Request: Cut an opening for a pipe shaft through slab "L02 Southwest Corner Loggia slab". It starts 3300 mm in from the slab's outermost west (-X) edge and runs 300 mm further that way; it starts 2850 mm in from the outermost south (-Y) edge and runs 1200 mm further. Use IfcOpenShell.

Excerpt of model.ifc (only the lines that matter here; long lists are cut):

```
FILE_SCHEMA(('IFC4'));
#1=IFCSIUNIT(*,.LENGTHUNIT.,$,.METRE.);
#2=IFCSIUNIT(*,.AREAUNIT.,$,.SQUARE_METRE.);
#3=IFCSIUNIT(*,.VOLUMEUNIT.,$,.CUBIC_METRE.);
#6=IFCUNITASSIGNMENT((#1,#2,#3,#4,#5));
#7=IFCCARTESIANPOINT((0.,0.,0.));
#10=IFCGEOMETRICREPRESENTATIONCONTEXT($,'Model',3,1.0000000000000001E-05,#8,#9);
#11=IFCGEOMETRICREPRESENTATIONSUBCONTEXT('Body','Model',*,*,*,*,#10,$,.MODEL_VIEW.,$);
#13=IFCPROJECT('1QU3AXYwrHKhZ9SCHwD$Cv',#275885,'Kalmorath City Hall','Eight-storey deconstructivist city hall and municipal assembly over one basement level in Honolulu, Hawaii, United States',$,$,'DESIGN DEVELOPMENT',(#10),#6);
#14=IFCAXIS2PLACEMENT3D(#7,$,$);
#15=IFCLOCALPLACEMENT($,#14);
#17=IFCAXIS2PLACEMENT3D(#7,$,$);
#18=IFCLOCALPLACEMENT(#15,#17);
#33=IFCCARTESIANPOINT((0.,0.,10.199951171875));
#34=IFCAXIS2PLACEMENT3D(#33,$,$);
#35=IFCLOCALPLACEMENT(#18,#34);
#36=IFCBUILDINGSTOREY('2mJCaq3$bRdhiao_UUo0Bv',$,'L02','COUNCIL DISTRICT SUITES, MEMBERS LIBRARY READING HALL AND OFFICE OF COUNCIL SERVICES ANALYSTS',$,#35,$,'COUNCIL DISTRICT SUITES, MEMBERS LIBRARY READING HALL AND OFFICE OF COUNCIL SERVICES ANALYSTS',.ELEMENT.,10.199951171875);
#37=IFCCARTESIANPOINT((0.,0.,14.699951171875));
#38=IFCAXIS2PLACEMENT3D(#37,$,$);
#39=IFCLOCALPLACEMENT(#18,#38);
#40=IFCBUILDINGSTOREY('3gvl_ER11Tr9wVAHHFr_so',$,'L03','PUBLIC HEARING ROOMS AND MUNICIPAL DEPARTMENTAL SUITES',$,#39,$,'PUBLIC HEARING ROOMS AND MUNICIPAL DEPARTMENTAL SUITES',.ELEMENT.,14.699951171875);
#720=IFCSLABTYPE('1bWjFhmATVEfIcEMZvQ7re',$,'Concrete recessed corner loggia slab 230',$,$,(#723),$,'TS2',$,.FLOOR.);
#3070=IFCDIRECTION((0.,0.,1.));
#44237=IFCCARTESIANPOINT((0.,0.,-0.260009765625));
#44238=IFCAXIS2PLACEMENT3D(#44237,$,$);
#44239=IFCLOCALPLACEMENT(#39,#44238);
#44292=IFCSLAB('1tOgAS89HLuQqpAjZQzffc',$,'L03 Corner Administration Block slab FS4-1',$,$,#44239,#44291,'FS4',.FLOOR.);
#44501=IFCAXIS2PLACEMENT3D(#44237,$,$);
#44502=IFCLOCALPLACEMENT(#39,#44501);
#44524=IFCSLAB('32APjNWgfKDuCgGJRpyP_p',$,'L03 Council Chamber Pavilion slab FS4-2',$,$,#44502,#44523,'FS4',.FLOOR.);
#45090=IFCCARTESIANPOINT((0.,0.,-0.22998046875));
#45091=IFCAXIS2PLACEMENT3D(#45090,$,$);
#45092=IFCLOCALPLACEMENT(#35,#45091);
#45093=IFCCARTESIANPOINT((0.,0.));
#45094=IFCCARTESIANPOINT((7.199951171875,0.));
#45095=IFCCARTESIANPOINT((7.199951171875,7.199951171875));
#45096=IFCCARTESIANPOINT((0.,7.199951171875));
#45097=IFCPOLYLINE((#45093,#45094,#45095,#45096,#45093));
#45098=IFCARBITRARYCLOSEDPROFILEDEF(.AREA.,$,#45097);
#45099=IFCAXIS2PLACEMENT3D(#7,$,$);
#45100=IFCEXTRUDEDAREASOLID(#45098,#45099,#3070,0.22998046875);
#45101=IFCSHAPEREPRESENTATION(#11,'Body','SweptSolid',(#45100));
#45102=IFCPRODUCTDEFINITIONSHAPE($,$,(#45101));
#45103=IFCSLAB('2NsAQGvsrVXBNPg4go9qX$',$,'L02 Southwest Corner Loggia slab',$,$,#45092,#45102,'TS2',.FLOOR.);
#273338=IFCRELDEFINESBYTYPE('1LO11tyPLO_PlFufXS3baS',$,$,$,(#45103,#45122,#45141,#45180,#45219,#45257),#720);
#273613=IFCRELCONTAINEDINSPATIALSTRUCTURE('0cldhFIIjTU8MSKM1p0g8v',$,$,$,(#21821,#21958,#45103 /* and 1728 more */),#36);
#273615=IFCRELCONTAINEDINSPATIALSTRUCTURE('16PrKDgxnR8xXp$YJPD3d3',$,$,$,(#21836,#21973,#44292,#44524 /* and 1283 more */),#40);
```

```python
import numpy as np
import ifcopenshell
import ifcopenshell.api.feature
import ifcopenshell.api.geometry
import ifcopenshell.api.root
import ifcopenshell.geom
import ifcopenshell.util.placement
import ifcopenshell.util.representation
import ifcopenshell.util.shape
import ifcopenshell.util.unit

model = ifcopenshell.open("model.ifc")
unit_scale = ifcopenshell.util.unit.calculate_unit_scale(model)
settings = ifcopenshell.geom.settings()


def volume(element):
    """Net volume in cubic metres, openings subtracted."""
    shape = ifcopenshell.geom.create_shape(settings, element)
    return ifcopenshell.util.shape.get_volume(shape.geometry)


slab = model.by_guid("2NsAQGvsrVXBNPg4go9qX$")
before = volume(slab)

# Extent in the slab's own axes, in metres. The edges named are its -X and -Y sides.
slab_shape = ifcopenshell.geom.create_shape(settings, slab)
vertices = ifcopenshell.util.shape.get_vertices(slab_shape.geometry)
x_min, y_min, bottom = vertices.min(axis=0)
top = vertices[:, 2].max()

opening = ifcopenshell.api.root.create_entity(model, ifc_class="IfcOpeningElement", name="Pipe shaft opening", predefined_type="OPENING")
context = ifcopenshell.util.representation.get_context(model, "Model", "Body", "MODEL_VIEW")
width, depth = 0.3, 1.2
outline = [(0.0, 0.0), (width, 0.0), (width, depth), (0.0, depth), (0.0, 0.0)]
# Overshoot both faces by 50 mm so the cut is clean.
shape = ifcopenshell.api.geometry.add_slab_representation(
    model, context=context, depth=top - bottom + 0.1, polyline=outline
)
ifcopenshell.api.geometry.assign_representation(model, product=opening, representation=shape)

matrix = ifcopenshell.util.placement.get_local_placement(slab.ObjectPlacement)
matrix[:, 3] = matrix @ np.append(np.array([x_min + 3.3, y_min + 2.85, bottom - 0.05]) / unit_scale, 1.0)
ifcopenshell.api.geometry.edit_object_placement(model, product=opening, matrix=matrix, is_si=False)
ifcopenshell.api.feature.add_feature(model, feature=opening, element=slab)

after = volume(slab)

print(f"slab volume {before:.3f} -> {after:.3f} m3")

model.write("model_edited.ifc")
```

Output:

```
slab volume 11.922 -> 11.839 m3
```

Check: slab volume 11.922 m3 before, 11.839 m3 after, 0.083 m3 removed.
